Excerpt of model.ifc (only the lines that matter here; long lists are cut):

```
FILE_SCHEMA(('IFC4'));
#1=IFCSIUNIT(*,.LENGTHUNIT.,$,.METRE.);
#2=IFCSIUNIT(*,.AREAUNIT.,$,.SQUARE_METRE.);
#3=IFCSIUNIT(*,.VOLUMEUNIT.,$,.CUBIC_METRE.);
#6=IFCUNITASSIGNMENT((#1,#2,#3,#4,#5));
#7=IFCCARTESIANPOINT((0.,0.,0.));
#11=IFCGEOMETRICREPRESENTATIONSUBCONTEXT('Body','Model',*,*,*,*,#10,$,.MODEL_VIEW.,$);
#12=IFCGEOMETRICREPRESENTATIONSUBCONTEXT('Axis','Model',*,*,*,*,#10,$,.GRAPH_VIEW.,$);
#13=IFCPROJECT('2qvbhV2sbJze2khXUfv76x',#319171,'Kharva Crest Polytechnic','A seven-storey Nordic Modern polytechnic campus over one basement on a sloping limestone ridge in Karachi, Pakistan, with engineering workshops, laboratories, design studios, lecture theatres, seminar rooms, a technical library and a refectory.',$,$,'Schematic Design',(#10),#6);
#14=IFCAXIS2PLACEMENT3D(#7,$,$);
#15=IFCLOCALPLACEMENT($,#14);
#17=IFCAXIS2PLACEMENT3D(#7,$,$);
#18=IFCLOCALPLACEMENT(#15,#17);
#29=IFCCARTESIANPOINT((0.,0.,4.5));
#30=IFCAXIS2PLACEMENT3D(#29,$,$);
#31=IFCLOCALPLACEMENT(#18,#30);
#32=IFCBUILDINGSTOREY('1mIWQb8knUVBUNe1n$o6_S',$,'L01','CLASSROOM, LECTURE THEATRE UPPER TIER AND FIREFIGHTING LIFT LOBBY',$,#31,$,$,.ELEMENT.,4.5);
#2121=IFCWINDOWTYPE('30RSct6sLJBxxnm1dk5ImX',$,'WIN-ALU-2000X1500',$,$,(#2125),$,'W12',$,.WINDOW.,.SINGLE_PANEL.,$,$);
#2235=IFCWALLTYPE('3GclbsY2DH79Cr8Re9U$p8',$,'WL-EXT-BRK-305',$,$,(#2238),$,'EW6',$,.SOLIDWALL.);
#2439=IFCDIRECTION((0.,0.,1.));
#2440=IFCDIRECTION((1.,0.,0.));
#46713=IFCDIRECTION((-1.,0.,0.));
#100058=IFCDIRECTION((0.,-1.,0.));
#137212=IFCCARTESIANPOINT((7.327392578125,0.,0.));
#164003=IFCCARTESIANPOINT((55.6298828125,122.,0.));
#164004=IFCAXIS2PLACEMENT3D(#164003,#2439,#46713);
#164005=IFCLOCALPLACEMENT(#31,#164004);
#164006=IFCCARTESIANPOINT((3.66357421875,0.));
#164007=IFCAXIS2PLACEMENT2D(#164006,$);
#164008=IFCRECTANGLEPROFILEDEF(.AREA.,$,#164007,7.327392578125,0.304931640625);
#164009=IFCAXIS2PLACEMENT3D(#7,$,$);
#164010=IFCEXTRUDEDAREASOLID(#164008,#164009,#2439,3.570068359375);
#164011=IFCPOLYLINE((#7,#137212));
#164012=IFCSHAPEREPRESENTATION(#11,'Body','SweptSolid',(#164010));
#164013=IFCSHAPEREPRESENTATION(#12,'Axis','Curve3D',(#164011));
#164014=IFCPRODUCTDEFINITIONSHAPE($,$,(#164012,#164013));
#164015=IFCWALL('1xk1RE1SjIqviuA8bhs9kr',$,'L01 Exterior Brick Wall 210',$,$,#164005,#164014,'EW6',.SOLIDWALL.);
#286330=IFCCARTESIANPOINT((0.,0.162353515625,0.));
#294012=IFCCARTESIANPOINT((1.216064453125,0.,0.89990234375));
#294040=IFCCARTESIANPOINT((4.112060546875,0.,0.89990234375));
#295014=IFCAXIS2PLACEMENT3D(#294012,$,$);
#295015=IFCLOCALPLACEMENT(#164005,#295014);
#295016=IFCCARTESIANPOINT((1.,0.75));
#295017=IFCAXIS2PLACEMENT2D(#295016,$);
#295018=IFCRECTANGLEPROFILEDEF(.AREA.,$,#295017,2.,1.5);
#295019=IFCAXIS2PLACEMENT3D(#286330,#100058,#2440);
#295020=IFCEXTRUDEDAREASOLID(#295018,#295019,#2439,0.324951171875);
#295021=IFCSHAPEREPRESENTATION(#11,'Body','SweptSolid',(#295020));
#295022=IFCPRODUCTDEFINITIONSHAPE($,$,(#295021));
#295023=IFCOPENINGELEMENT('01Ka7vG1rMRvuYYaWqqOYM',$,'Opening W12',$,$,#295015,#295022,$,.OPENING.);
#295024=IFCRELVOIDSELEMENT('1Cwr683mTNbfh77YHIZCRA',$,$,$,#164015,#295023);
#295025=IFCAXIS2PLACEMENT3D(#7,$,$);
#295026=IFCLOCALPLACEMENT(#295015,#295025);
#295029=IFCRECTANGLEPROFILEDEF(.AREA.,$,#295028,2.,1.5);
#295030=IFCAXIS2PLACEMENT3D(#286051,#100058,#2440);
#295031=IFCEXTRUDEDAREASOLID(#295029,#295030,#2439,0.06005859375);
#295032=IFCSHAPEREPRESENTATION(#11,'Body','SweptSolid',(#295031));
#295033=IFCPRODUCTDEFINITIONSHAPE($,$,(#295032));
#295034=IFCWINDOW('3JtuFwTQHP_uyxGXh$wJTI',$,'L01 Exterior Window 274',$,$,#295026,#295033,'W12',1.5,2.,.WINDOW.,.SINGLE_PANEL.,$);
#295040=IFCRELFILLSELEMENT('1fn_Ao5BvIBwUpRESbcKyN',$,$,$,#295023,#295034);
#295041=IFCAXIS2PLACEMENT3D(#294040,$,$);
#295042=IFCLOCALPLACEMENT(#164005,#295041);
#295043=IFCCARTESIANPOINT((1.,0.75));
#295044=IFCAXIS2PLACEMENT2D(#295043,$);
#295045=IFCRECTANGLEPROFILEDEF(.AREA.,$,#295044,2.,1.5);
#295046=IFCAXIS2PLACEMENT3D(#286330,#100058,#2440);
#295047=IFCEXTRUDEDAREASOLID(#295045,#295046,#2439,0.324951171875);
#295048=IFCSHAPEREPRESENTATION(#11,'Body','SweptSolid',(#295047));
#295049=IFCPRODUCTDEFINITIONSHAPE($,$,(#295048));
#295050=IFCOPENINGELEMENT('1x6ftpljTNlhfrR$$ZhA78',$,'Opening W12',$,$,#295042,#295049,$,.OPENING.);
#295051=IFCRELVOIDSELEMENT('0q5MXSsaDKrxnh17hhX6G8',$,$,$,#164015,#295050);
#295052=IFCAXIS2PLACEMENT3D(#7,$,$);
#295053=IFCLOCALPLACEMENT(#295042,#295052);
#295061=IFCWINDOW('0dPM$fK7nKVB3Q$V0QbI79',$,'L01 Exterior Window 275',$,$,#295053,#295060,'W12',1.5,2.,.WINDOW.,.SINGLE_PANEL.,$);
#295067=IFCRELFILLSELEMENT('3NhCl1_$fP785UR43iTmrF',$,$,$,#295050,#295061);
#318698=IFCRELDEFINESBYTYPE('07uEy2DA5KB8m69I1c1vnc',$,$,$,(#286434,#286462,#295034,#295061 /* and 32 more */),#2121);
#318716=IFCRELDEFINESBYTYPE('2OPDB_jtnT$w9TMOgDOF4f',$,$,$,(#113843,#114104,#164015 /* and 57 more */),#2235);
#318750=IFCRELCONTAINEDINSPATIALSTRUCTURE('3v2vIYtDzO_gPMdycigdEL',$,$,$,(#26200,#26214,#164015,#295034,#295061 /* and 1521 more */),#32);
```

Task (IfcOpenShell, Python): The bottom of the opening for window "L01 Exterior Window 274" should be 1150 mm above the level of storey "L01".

```python
import numpy as np
import ifcopenshell
import ifcopenshell.api.geometry
import ifcopenshell.geom
import ifcopenshell.util.element
import ifcopenshell.util.placement
import ifcopenshell.util.shape
import ifcopenshell.util.unit

model = ifcopenshell.open("model.ifc")
unit_scale = ifcopenshell.util.unit.calculate_unit_scale(model)

window = model.by_id(295034)
opening = window.FillsVoids[0].RelatingOpeningElement
storey = ifcopenshell.util.element.get_container(window, ifc_class="IfcBuildingStorey")
level = ifcopenshell.util.placement.get_local_placement(storey.ObjectPlacement)[2, 3]

# The opening's origin need not be at the sill, so measure its lowest point.
shape = ifcopenshell.geom.create_shape(ifcopenshell.geom.settings(), opening)
bottom = ifcopenshell.util.shape.get_shape_bottom_elevation(shape, shape.geometry) / unit_scale
dz = level + 1.15 / unit_scale - bottom

shift = np.array([0.0, 0.0, dz])
# The window is placed relative to its opening, so it follows when the opening moves.
matrix = ifcopenshell.util.placement.get_local_placement(opening.ObjectPlacement)
matrix[:3, 3] += shift
ifcopenshell.api.geometry.edit_object_placement(
    model, product=opening, matrix=matrix, is_si=False, should_transform_children=True
)

print(f"moved by {dz * unit_scale:+.3f} m")

model.write("model_v2.ifc")
```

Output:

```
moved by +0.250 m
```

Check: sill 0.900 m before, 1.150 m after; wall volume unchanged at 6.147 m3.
